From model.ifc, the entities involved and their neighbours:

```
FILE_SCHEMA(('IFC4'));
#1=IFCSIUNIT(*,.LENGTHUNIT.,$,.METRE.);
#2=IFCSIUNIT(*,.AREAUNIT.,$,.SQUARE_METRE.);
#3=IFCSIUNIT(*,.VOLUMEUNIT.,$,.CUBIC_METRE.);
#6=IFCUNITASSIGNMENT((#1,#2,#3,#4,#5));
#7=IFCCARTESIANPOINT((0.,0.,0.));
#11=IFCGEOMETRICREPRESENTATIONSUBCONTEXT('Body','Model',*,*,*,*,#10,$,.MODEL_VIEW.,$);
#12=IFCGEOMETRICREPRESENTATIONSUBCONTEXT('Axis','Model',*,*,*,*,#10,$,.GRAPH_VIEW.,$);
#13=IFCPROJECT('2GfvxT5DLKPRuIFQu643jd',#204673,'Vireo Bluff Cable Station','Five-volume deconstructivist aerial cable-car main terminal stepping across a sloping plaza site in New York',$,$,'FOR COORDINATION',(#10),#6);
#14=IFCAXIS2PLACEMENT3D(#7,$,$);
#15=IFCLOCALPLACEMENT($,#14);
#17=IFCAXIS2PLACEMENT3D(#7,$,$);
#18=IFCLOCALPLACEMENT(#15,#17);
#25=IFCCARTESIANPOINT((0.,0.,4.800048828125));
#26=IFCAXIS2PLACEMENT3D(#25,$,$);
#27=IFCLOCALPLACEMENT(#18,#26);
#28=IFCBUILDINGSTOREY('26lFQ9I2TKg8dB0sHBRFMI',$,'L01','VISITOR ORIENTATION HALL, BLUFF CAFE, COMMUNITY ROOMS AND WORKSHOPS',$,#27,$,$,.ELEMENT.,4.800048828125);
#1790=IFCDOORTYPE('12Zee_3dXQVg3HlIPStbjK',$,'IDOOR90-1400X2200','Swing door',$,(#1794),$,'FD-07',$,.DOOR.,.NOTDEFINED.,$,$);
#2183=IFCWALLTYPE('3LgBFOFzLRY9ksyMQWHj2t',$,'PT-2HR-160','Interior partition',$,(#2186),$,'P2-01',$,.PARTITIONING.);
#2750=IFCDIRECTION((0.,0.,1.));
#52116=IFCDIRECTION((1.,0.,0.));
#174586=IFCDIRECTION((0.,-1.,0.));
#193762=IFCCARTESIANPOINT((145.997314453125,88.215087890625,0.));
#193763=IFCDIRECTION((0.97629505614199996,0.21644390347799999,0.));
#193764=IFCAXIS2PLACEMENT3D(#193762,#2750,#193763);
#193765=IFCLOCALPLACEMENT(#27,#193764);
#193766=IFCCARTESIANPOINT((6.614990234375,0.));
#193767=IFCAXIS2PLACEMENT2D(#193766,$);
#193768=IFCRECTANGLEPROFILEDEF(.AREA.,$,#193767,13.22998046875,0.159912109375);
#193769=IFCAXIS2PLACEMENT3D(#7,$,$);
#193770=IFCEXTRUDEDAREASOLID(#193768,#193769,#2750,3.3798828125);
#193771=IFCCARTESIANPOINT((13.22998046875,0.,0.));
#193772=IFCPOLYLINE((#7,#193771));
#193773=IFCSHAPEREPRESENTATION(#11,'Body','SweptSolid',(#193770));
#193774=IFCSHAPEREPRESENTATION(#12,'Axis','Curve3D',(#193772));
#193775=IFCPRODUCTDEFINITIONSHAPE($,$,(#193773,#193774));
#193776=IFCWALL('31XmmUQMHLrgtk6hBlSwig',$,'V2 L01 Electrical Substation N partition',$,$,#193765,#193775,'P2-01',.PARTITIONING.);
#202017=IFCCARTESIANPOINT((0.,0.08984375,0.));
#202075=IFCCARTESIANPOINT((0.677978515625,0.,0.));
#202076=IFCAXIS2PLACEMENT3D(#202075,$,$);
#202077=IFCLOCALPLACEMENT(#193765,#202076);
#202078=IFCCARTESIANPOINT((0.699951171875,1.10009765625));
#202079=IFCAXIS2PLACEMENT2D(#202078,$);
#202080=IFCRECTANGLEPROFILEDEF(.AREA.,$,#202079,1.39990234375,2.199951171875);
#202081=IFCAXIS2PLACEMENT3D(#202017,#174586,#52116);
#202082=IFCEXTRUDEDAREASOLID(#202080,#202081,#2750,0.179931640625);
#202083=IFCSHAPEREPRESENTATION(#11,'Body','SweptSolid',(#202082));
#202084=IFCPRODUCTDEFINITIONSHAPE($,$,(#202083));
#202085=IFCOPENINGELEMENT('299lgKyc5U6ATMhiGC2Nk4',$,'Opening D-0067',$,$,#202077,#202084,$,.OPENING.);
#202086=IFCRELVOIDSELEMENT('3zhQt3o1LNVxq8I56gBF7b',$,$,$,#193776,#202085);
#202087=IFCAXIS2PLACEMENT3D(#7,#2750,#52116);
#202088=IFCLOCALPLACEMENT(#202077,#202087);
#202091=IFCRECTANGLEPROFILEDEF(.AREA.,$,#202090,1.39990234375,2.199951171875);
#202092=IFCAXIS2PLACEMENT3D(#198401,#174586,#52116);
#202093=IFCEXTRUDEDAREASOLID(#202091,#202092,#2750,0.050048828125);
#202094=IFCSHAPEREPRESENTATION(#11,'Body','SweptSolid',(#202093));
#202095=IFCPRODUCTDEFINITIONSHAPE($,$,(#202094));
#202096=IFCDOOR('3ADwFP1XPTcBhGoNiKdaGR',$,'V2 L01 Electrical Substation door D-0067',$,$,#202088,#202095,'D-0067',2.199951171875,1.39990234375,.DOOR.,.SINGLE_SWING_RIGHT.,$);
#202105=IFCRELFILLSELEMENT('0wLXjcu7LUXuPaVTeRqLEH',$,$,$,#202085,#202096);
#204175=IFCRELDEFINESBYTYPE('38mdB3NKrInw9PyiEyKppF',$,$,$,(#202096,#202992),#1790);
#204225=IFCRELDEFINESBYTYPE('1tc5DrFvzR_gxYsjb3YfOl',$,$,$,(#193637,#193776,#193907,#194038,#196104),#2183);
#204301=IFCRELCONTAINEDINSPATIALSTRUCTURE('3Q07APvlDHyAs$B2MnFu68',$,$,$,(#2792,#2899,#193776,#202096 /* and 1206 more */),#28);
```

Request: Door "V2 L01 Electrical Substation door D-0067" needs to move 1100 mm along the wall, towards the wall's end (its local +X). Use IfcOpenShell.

```python
import ifcopenshell
import ifcopenshell.api.geometry
import ifcopenshell.util.placement
import ifcopenshell.util.unit

model = ifcopenshell.open("model.ifc")
unit_scale = ifcopenshell.util.unit.calculate_unit_scale(model)

door = model.by_id(202096)
opening = door.FillsVoids[0].RelatingOpeningElement
wall = opening.VoidsElements[0].RelatingBuildingElement

wall_matrix = ifcopenshell.util.placement.get_local_placement(wall.ObjectPlacement)
shift = wall_matrix[:3, 0] * 1.1 / unit_scale
before = ifcopenshell.util.placement.get_local_placement(door.ObjectPlacement)[:3, 3].copy()

# The door is placed relative to its opening, so it follows when the opening moves.
matrix = ifcopenshell.util.placement.get_local_placement(opening.ObjectPlacement)
matrix[:3, 3] += shift
ifcopenshell.api.geometry.edit_object_placement(
    model, product=opening, matrix=matrix, is_si=False, should_transform_children=True
)

after = ifcopenshell.util.placement.get_local_placement(door.ObjectPlacement)[:3, 3]
print("door moved by", (after - before).round(3) + 0.0)

model.write("model-out.ifc")
```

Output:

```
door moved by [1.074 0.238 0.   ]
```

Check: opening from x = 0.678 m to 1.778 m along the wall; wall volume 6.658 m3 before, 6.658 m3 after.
